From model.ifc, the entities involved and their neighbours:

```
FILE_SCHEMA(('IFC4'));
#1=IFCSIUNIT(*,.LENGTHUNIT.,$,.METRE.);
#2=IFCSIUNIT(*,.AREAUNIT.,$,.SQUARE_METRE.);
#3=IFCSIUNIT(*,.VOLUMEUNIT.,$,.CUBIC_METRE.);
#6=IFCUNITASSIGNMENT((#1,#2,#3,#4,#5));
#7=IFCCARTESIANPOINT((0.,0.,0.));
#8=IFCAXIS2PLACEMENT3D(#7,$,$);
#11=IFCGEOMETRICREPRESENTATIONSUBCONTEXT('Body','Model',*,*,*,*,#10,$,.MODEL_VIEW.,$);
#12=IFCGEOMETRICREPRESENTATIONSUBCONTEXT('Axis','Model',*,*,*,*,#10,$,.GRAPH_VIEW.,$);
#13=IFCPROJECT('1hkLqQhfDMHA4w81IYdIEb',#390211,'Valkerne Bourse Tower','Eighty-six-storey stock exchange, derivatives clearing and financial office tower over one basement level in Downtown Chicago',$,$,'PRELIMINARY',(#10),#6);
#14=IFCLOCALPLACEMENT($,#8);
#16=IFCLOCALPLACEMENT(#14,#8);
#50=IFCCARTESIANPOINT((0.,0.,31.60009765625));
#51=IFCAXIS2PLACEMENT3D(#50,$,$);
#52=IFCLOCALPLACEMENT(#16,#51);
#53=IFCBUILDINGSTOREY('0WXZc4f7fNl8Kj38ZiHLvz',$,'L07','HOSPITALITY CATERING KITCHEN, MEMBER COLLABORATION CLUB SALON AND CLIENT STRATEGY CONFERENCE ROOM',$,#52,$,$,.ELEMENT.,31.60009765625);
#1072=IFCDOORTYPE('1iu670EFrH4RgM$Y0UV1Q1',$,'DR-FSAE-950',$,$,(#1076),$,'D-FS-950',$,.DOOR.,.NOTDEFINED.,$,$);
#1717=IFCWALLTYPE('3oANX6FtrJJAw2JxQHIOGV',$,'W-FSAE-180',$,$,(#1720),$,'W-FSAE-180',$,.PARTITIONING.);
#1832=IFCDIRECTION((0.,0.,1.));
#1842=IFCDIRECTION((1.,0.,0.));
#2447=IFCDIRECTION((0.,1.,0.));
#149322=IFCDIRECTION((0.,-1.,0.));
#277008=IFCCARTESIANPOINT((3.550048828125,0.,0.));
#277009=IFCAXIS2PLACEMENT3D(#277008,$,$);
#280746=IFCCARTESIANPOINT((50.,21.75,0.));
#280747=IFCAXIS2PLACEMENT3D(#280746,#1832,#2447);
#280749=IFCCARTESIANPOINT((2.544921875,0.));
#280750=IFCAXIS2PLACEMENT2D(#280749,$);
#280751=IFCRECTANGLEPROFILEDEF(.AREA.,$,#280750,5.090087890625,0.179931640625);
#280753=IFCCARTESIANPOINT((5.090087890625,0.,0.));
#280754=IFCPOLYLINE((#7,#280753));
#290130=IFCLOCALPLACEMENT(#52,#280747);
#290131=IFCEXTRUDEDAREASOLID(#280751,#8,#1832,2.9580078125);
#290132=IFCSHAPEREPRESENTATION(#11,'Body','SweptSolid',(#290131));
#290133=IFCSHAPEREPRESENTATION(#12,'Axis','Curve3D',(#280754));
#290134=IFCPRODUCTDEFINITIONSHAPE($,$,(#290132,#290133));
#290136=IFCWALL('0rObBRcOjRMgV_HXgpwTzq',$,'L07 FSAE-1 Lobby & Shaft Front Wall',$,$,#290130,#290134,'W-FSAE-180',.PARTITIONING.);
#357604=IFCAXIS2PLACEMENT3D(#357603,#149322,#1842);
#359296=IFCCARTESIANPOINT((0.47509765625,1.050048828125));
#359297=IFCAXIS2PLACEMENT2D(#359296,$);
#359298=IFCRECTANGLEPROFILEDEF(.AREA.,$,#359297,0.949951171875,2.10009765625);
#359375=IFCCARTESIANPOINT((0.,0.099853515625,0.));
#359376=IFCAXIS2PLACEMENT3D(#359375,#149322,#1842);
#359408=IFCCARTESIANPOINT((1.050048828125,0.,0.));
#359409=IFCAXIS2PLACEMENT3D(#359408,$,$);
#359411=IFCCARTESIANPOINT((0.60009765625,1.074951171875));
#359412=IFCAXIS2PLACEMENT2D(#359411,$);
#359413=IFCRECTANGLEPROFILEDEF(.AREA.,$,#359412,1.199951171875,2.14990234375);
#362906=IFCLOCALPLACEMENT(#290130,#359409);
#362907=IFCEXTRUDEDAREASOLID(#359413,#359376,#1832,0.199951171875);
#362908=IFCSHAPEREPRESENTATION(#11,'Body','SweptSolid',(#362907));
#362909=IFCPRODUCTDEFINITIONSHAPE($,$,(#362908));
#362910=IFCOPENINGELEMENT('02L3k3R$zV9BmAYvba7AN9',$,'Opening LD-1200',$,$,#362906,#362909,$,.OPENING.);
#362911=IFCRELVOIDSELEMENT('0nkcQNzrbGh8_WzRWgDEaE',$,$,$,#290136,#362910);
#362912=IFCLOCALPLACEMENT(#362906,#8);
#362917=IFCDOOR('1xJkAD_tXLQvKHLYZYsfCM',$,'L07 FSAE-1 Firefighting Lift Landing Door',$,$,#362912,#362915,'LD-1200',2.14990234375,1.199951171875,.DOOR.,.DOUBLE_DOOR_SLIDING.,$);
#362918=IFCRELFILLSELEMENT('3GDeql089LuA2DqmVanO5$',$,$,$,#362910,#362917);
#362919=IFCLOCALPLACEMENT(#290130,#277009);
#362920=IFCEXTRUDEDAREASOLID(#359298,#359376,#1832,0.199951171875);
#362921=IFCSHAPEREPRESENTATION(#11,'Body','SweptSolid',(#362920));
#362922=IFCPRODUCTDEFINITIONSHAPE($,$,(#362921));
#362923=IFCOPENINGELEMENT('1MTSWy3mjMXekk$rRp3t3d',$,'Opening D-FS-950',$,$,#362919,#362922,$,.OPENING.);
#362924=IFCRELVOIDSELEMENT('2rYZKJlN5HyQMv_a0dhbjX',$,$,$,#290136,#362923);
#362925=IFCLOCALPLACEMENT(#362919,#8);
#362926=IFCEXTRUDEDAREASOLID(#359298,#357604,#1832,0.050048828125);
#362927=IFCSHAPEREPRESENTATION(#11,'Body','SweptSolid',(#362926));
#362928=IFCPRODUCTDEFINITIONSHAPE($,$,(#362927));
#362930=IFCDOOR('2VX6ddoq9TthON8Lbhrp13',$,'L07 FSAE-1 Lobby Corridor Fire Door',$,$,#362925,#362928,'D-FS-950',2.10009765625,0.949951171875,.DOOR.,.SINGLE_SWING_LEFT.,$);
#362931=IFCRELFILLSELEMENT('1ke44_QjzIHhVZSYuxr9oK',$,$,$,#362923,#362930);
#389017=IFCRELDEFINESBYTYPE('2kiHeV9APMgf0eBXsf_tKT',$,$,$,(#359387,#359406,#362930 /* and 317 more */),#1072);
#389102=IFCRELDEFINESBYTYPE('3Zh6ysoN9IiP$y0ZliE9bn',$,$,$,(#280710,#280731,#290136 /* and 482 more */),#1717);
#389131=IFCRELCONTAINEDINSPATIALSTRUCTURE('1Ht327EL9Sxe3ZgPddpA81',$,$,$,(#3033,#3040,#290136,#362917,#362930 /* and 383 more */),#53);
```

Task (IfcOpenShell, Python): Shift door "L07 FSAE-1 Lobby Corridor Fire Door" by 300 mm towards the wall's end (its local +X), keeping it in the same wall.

```python
import ifcopenshell
import ifcopenshell.api.geometry
import ifcopenshell.util.placement

model = ifcopenshell.open("model.ifc")

door = model.by_guid("2VX6ddoq9TthON8Lbhrp13")
opening = door.FillsVoids[0].RelatingOpeningElement
wall = opening.VoidsElements[0].RelatingBuildingElement

wall_matrix = ifcopenshell.util.placement.get_local_placement(wall.ObjectPlacement)
shift = wall_matrix[:3, 0] * 0.3
before = ifcopenshell.util.placement.get_local_placement(door.ObjectPlacement)[:3, 3].copy()

# The door is placed relative to its opening, so it follows when the opening moves.
matrix = ifcopenshell.util.placement.get_local_placement(opening.ObjectPlacement)
matrix[:3, 3] += shift
ifcopenshell.api.geometry.edit_object_placement(
    model, product=opening, matrix=matrix, is_si=False, should_transform_children=True
)

after = ifcopenshell.util.placement.get_local_placement(door.ObjectPlacement)[:3, 3]
print("door moved by", (after - before).round(3) + 0.0)

model.write("model_v2.ifc")
```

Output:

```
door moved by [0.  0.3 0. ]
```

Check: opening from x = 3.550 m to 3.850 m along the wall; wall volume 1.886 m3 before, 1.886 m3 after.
